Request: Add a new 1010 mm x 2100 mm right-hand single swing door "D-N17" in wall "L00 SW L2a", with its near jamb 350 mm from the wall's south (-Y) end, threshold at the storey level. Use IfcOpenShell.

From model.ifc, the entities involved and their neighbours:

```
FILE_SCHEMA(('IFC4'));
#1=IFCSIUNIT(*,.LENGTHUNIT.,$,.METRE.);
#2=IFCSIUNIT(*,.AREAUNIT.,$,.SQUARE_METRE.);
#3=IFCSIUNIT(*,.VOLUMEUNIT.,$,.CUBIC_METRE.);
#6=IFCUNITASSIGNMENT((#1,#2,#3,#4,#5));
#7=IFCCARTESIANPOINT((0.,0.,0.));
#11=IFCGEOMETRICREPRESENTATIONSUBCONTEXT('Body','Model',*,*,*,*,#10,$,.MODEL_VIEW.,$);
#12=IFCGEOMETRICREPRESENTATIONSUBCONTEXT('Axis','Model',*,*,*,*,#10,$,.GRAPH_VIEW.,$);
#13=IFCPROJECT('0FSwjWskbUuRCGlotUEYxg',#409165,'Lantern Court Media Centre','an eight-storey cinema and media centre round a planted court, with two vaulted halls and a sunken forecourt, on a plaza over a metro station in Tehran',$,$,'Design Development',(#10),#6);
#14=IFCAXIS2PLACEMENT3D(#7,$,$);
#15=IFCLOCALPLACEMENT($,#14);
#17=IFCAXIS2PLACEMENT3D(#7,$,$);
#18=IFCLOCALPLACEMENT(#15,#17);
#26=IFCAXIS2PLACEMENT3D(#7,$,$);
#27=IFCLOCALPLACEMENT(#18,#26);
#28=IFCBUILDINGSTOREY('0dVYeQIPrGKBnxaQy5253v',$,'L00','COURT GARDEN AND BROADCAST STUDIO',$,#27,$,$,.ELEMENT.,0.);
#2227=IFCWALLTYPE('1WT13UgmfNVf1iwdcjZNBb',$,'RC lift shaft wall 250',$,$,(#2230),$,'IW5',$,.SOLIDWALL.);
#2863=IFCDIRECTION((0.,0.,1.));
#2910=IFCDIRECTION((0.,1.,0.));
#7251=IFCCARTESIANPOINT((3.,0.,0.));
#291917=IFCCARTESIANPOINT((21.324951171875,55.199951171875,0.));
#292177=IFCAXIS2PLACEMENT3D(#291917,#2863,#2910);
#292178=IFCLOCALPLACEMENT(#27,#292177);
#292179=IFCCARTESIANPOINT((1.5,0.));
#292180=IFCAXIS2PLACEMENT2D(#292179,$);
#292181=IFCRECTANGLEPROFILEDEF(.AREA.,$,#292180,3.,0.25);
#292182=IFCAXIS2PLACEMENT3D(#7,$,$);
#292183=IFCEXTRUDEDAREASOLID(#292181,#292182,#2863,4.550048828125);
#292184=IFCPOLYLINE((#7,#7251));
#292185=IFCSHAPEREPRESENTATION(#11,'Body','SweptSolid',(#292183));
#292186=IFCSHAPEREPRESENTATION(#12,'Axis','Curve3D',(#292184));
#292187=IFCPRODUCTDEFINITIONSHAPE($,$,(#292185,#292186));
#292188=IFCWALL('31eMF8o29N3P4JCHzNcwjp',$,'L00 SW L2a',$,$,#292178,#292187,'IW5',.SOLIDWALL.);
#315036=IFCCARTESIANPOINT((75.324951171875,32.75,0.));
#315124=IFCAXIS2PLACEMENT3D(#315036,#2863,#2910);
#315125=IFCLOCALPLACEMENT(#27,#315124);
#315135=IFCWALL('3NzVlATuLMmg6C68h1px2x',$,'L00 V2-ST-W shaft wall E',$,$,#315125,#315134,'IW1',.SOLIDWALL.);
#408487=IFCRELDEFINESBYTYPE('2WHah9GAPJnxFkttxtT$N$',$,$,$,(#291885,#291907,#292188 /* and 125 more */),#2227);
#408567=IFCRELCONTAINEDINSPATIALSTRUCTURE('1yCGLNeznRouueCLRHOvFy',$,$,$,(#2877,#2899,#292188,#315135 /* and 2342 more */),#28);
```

```python
import numpy as np
import ifcopenshell
import ifcopenshell.api.feature
import ifcopenshell.api.geometry
import ifcopenshell.api.root
import ifcopenshell.api.spatial
import ifcopenshell.geom
import ifcopenshell.util.element
import ifcopenshell.util.placement
import ifcopenshell.util.representation
import ifcopenshell.util.shape
import ifcopenshell.util.unit

model = ifcopenshell.open("model.ifc")
unit_scale = ifcopenshell.util.unit.calculate_unit_scale(model)
settings = ifcopenshell.geom.settings()


def volume(element):
    """Net volume in cubic metres, openings subtracted."""
    shape = ifcopenshell.geom.create_shape(settings, element)
    return ifcopenshell.util.shape.get_volume(shape.geometry)


wall = model.by_id(292188)
storey = ifcopenshell.util.element.get_container(wall, ifc_class="IfcBuildingStorey")
context = ifcopenshell.util.representation.get_context(model, "Model", "Body", "MODEL_VIEW")
before = volume(wall)

width, height, from_end, sill = 1.01, 2.1, 0.35, 0.0  # metres

# The wall runs along its own X axis, and the end named is its -X end.
wall_shape = ifcopenshell.geom.create_shape(settings, wall)
x, y, z = ifcopenshell.util.shape.get_vertices(wall_shape.geometry).T
start = x.min() + from_end
face, thickness = float(y.min()), float(y.max() - y.min())
wall_matrix = ifcopenshell.util.placement.get_local_placement(wall.ObjectPlacement)
level = ifcopenshell.util.placement.get_local_placement(storey.ObjectPlacement)[2, 3]


def in_wall(x, y):
    """Placement at x, y metres in the wall's axes, at sill height."""
    matrix = wall_matrix.copy()
    matrix[:, 3] = wall_matrix @ np.array([x / unit_scale, y / unit_scale, 0.0, 1.0])
    matrix[2, 3] = level + sill / unit_scale
    return matrix


# Opening: a box that overshoots both wall faces by 50 mm.
opening = ifcopenshell.api.root.create_entity(model, ifc_class="IfcOpeningElement", predefined_type="OPENING")
box = ifcopenshell.api.geometry.add_wall_representation(
    model, context=context, length=width, height=height, thickness=thickness + 0.1
)
ifcopenshell.api.geometry.assign_representation(model, product=opening, representation=box)
ifcopenshell.api.geometry.edit_object_placement(model, product=opening, matrix=in_wall(start, face - 0.05), is_si=False)
ifcopenshell.api.feature.add_feature(model, feature=opening, element=wall)

door = ifcopenshell.api.root.create_entity(model, ifc_class="IfcDoor", name="D-N17", predefined_type="DOOR")
door.OverallWidth, door.OverallHeight = width / unit_scale, height / unit_scale
door.OperationType = "SINGLE_SWING_RIGHT"
body = ifcopenshell.api.geometry.add_door_representation(
    model,
    context=context,
    overall_width=door.OverallWidth,
    overall_height=door.OverallHeight,
    operation_type="SINGLE_SWING_RIGHT",
    lining_properties={"LiningDepth": thickness / unit_scale, "ThresholdDepth": thickness / unit_scale},
)
ifcopenshell.api.geometry.assign_representation(model, product=door, representation=body)
ifcopenshell.api.spatial.assign_container(model, products=[door], relating_structure=storey)
ifcopenshell.api.feature.add_filling(model, opening=opening, element=door)

# The lining spans the wall, so the door starts at the wall face.
ifcopenshell.api.geometry.edit_object_placement(model, product=door, matrix=in_wall(start, face), is_si=False)

after = volume(wall)

print(f"wall volume {before:.3f} -> {after:.3f} m3")

model.write("model_rev.ifc")
```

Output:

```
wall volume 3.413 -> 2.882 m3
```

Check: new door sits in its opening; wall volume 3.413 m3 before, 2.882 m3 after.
